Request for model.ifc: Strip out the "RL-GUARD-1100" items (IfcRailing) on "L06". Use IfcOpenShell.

First a look at what the model holds.

```python
import ifcopenshell
import ifcopenshell.util.element

model = ifcopenshell.open("model.ifc")
print(model.schema)
storey = next(s for s in model.by_type("IfcBuildingStorey") if s.Name == "L06")
railings = [e for e in ifcopenshell.util.element.get_decomposition(storey) if e.is_a("IfcRailing")]
seen = {}
for e in railings:
    element_type = ifcopenshell.util.element.get_type(e)
    name = element_type.Name if element_type not in (None, e) else None
    seen[name] = seen.get(name, 0) + 1
for name, count in sorted(seen.items(), key=str):
    print(count, "x", name)
```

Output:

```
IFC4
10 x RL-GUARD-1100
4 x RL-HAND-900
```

```python
import ifcopenshell
import ifcopenshell.api.root
import ifcopenshell.util.element

model = ifcopenshell.open("model.ifc")

storey = next(s for s in model.by_type("IfcBuildingStorey") if s.Name == "L06")
railings = [e for e in ifcopenshell.util.element.get_decomposition(storey) if e.is_a("IfcRailing")]
targets = [e for e in railings if (t := ifcopenshell.util.element.get_type(e)) not in (None, e) and t.Name == "RL-GUARD-1100"]

for e in targets:
    ifcopenshell.api.root.remove_product(model, product=e)
print(len(targets), "removed")

model.write("model_v2.ifc")
```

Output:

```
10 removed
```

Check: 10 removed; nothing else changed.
